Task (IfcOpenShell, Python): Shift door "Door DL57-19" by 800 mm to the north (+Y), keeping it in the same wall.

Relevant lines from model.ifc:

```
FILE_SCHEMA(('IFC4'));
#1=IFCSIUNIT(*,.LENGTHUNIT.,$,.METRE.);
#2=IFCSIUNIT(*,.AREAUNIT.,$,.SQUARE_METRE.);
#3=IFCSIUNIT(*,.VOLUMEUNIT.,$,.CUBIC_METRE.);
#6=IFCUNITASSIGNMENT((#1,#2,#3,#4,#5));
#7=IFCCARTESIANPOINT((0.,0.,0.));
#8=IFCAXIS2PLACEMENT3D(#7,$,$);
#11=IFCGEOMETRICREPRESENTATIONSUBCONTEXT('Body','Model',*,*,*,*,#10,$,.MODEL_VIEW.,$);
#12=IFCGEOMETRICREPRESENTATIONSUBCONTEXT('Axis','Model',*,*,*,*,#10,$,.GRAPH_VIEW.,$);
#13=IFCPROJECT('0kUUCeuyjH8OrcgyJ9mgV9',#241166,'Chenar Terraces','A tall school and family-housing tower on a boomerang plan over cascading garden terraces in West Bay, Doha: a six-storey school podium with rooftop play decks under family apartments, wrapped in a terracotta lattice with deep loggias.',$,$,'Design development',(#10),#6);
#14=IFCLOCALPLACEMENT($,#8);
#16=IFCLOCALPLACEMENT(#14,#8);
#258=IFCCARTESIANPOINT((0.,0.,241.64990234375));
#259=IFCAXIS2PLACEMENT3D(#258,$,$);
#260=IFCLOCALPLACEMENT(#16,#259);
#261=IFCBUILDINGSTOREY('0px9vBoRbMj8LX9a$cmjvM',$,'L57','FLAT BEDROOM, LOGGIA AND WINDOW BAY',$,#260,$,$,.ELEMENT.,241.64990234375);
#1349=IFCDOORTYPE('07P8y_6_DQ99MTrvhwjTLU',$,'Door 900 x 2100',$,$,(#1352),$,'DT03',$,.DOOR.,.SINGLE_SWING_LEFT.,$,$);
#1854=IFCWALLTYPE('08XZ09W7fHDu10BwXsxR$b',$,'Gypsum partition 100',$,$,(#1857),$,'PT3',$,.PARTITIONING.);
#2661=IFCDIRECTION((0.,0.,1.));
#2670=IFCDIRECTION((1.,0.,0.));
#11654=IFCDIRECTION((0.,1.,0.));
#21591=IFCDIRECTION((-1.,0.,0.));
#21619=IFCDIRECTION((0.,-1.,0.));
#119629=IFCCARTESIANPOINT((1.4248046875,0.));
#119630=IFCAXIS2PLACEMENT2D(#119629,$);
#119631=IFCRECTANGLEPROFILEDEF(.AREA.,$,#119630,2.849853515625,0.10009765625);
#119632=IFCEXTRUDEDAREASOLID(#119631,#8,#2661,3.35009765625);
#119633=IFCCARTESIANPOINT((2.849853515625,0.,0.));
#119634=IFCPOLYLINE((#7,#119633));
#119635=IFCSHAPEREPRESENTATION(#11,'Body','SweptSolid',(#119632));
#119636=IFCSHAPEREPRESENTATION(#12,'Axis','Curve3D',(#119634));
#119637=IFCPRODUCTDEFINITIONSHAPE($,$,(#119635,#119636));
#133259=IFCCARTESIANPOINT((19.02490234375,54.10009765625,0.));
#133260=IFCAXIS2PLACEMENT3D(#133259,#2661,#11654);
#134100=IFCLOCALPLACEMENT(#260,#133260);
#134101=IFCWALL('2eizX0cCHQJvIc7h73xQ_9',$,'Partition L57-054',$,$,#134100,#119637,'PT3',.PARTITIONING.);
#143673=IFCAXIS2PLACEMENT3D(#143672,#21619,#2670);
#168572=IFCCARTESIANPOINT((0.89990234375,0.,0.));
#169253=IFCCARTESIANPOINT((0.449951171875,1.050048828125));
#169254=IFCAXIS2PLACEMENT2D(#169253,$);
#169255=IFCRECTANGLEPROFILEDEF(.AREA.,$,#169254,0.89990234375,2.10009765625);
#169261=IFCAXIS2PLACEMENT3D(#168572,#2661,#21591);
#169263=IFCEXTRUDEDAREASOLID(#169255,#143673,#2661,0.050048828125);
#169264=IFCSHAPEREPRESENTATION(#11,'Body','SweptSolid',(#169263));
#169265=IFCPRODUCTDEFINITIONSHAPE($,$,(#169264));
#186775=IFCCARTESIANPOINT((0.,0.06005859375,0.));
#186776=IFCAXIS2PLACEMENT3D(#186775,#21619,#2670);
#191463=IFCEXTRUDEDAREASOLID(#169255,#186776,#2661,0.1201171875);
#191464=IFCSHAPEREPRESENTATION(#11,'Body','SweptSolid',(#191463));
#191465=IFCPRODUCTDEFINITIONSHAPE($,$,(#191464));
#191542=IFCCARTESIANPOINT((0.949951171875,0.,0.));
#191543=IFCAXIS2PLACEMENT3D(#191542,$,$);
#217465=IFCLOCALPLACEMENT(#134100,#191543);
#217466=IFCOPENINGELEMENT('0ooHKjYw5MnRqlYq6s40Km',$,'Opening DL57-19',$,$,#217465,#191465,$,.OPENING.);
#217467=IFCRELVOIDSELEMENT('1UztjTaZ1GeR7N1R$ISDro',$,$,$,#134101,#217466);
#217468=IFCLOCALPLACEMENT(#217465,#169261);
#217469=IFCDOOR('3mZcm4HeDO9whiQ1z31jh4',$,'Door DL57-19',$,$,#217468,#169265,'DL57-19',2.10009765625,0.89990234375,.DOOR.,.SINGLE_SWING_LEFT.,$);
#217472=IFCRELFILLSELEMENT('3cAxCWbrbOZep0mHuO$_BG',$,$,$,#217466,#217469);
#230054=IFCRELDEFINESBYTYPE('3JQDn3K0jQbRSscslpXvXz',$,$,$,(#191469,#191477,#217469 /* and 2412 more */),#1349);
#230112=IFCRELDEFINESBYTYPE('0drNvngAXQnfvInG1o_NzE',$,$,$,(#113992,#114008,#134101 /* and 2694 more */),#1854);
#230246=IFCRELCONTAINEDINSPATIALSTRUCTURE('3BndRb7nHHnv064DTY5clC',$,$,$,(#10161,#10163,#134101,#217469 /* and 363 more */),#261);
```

```python
import ifcopenshell
import ifcopenshell.api.geometry
import ifcopenshell.util.placement

model = ifcopenshell.open("model.ifc")

door = model.by_guid("3mZcm4HeDO9whiQ1z31jh4")
opening = door.FillsVoids[0].RelatingOpeningElement
wall = opening.VoidsElements[0].RelatingBuildingElement

wall_matrix = ifcopenshell.util.placement.get_local_placement(wall.ObjectPlacement)
shift = wall_matrix[:3, 0] * 0.8
before = ifcopenshell.util.placement.get_local_placement(door.ObjectPlacement)[:3, 3].copy()

# The door is placed relative to its opening, so it follows when the opening moves.
matrix = ifcopenshell.util.placement.get_local_placement(opening.ObjectPlacement)
matrix[:3, 3] += shift
ifcopenshell.api.geometry.edit_object_placement(
    model, product=opening, matrix=matrix, is_si=False, should_transform_children=True
)

after = ifcopenshell.util.placement.get_local_placement(door.ObjectPlacement)[:3, 3]
print("door moved by", (after - before).round(3) + 0.0)

model.write("model_edited.ifc")
```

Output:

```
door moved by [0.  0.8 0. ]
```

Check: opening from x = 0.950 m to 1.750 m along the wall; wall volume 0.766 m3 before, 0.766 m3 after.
